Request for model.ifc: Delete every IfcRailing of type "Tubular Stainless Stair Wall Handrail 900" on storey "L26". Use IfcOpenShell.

First a look at what the model holds.

```python
import ifcopenshell
import ifcopenshell.util.element

model = ifcopenshell.open("model.ifc")
print(model.schema)
storey = next(s for s in model.by_type("IfcBuildingStorey") if s.Name == "L26")
railings = [e for e in ifcopenshell.util.element.get_decomposition(storey) if e.is_a("IfcRailing")]
seen = {}
for e in railings:
    element_type = ifcopenshell.util.element.get_type(e)
    name = element_type.Name if element_type not in (None, e) else None
    seen[name] = seen.get(name, 0) + 1
for name, count in sorted(seen.items(), key=str):
    print(count, "x", name)
```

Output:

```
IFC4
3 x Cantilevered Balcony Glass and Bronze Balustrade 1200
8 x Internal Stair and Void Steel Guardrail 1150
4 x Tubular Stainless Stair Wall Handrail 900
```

```python
import ifcopenshell
import ifcopenshell.api.root
import ifcopenshell.util.element

model = ifcopenshell.open("model.ifc")

storey = next(s for s in model.by_type("IfcBuildingStorey") if s.Name == "L26")
railings = [e for e in ifcopenshell.util.element.get_decomposition(storey) if e.is_a("IfcRailing")]
targets = [e for e in railings if (t := ifcopenshell.util.element.get_type(e)) not in (None, e) and t.Name == "Tubular Stainless Stair Wall Handrail 900"]

for e in targets:
    ifcopenshell.api.root.remove_product(model, product=e)
print(len(targets), "removed")

model.write("model_edited.ifc")
```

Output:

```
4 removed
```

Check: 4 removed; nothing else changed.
